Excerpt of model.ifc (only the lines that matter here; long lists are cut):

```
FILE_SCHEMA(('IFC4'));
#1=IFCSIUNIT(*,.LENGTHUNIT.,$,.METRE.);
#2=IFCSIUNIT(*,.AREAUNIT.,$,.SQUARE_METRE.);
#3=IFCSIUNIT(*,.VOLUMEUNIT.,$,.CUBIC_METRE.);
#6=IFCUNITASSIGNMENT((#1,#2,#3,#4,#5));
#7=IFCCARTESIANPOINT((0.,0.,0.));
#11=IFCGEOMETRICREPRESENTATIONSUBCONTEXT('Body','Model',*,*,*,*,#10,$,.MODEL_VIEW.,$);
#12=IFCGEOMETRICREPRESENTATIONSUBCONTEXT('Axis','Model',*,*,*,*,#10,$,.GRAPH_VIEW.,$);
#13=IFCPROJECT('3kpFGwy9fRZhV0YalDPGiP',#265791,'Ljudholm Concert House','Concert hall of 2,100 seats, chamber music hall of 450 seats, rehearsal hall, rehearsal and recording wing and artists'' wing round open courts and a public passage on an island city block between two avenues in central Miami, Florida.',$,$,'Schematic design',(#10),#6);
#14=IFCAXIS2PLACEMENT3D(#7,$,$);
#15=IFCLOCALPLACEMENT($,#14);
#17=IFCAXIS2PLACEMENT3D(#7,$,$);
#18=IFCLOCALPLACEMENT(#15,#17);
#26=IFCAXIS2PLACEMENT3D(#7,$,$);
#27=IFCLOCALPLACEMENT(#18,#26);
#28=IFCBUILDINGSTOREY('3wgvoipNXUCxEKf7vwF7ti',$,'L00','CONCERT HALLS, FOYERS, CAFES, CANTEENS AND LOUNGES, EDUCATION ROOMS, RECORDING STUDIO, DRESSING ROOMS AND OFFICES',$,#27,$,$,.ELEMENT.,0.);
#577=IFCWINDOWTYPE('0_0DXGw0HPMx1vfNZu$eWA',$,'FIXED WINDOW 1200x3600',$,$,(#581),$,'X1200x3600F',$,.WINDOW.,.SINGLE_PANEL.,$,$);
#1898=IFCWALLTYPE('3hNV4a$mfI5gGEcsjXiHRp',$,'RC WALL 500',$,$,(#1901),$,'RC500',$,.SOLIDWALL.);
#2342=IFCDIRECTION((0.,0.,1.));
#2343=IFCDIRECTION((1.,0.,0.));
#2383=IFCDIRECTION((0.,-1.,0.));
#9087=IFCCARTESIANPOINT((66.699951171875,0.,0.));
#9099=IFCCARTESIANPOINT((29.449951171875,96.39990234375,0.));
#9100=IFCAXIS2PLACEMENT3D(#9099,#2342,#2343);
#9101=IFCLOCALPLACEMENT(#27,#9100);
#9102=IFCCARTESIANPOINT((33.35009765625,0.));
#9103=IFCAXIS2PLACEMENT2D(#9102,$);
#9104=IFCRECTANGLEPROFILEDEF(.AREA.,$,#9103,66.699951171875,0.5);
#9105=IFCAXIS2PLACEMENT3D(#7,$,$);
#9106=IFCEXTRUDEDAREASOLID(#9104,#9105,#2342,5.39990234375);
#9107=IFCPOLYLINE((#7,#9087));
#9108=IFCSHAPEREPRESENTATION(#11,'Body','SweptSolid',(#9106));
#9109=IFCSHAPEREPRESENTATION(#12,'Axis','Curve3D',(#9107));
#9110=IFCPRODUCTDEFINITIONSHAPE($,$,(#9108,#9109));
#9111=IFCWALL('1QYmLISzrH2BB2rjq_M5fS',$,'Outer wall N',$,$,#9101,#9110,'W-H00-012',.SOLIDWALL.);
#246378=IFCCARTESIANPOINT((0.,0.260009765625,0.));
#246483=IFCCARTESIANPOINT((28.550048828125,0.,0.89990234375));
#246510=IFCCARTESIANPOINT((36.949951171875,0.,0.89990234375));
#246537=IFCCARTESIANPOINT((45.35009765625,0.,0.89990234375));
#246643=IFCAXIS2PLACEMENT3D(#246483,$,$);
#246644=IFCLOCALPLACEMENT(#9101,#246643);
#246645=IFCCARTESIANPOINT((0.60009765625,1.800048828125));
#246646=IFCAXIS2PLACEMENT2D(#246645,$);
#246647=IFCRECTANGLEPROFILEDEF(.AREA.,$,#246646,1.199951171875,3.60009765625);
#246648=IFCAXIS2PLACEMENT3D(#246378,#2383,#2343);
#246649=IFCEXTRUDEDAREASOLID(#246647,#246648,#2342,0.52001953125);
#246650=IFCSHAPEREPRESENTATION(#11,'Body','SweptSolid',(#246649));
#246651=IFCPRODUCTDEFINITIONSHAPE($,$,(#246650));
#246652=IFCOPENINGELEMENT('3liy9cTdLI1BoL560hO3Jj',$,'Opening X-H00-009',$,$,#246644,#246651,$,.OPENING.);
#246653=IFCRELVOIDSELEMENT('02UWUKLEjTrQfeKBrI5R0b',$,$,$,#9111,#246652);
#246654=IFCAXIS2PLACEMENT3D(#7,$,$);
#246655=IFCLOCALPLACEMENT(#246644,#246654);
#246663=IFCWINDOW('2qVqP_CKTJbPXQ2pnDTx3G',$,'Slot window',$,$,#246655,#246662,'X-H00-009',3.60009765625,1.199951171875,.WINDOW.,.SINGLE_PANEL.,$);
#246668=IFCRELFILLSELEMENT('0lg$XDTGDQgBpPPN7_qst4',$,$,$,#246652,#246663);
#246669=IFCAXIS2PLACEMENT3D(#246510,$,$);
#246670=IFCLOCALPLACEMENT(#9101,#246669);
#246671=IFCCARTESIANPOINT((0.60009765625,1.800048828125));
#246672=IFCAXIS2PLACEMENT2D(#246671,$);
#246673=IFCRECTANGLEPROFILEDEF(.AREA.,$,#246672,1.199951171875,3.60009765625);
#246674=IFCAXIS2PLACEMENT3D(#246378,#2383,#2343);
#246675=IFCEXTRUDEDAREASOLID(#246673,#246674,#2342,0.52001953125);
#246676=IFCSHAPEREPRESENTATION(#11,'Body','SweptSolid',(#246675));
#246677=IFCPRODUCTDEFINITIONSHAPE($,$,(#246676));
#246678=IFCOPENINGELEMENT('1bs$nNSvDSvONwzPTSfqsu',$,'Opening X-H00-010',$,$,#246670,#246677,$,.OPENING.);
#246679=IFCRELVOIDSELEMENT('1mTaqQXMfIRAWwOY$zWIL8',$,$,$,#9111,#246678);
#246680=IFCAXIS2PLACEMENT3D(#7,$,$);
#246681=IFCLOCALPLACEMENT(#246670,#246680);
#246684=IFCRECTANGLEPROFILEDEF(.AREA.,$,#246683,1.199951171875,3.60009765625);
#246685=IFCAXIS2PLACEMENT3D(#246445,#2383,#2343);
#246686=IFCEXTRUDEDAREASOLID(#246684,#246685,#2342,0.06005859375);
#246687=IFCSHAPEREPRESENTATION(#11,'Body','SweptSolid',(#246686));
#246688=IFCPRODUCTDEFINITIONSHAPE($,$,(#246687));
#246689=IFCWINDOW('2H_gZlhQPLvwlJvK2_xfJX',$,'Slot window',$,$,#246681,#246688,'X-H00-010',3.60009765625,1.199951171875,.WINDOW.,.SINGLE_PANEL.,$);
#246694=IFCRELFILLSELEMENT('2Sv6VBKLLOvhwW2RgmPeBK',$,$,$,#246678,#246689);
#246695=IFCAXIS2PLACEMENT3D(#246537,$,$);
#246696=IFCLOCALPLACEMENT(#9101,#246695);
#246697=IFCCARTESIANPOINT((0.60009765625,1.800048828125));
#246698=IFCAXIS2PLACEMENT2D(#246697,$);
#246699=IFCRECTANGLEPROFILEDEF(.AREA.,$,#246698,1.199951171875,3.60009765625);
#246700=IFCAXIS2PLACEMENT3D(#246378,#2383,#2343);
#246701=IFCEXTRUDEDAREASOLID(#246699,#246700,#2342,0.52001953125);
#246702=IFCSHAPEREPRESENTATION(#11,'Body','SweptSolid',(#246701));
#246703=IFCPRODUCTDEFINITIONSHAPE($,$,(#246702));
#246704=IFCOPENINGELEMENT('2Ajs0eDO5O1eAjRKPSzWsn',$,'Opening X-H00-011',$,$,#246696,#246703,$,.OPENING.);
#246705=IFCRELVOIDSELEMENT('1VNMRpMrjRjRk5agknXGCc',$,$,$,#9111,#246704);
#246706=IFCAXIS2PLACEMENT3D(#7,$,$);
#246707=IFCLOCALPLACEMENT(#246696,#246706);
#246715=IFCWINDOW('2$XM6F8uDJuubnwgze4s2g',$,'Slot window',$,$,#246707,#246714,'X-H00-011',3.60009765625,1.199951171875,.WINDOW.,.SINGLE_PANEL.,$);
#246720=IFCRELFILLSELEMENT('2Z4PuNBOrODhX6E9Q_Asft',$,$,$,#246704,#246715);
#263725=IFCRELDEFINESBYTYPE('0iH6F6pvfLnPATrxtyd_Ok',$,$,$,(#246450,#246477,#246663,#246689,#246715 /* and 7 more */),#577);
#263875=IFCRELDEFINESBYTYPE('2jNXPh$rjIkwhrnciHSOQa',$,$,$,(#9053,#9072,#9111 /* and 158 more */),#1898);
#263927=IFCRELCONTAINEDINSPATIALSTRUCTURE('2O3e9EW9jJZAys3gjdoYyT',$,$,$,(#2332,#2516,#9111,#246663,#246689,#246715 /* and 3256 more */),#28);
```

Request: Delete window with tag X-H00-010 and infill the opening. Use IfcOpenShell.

```python
import ifcopenshell
import ifcopenshell.api.feature
import ifcopenshell.api.root
import ifcopenshell.geom
import ifcopenshell.util.shape

model = ifcopenshell.open("model.ifc")
settings = ifcopenshell.geom.settings()


def volume(element):
    """Net volume in cubic metres, openings subtracted."""
    shape = ifcopenshell.geom.create_shape(settings, element)
    return ifcopenshell.util.shape.get_volume(shape.geometry)


window = model.by_guid("2H_gZlhQPLvwlJvK2_xfJX")
opening = window.FillsVoids[0].RelatingOpeningElement
wall = opening.VoidsElements[0].RelatingBuildingElement
before = volume(wall)

ifcopenshell.api.root.remove_product(model, product=window)
ifcopenshell.api.feature.remove_feature(model, feature=opening)

after = volume(wall)

print(f"wall volume {before:.3f} -> {after:.3f} m3")

model.write("model-out.ifc")
```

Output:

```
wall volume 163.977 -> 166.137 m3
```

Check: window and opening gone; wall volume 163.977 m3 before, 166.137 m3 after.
